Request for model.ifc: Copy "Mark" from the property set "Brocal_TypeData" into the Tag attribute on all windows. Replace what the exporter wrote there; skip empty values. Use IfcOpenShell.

First a look at what the model holds.

```python
import ifcopenshell
import ifcopenshell.util.element

model = ifcopenshell.open("model.ifc")
print(model.schema)
windows = model.by_type("IfcWindow")
print(len(windows), "windows")
for e in windows[:8]:
    source = ifcopenshell.util.element.get_pset(e, "Brocal_TypeData", "Mark")
    target = e.Tag
    print(e.id(), repr(source), repr(target), sep=" | ")
```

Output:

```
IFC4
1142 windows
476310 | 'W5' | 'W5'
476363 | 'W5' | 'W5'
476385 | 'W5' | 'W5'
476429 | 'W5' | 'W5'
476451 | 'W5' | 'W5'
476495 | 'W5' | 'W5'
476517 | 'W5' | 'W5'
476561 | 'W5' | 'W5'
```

```python
import ifcopenshell
import ifcopenshell.util.element

model = ifcopenshell.open("model.ifc")

count = 0
for e in model.by_type("IfcWindow"):
    value = ifcopenshell.util.element.get_pset(e, "Brocal_TypeData", "Mark")
    current = e.Tag
    if not value or not value.strip() or current == value:
        continue
    e.Tag = value
    count += 1

print(count, "windows updated")

model.write("model_edited.ifc")
```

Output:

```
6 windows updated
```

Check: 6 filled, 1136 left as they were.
